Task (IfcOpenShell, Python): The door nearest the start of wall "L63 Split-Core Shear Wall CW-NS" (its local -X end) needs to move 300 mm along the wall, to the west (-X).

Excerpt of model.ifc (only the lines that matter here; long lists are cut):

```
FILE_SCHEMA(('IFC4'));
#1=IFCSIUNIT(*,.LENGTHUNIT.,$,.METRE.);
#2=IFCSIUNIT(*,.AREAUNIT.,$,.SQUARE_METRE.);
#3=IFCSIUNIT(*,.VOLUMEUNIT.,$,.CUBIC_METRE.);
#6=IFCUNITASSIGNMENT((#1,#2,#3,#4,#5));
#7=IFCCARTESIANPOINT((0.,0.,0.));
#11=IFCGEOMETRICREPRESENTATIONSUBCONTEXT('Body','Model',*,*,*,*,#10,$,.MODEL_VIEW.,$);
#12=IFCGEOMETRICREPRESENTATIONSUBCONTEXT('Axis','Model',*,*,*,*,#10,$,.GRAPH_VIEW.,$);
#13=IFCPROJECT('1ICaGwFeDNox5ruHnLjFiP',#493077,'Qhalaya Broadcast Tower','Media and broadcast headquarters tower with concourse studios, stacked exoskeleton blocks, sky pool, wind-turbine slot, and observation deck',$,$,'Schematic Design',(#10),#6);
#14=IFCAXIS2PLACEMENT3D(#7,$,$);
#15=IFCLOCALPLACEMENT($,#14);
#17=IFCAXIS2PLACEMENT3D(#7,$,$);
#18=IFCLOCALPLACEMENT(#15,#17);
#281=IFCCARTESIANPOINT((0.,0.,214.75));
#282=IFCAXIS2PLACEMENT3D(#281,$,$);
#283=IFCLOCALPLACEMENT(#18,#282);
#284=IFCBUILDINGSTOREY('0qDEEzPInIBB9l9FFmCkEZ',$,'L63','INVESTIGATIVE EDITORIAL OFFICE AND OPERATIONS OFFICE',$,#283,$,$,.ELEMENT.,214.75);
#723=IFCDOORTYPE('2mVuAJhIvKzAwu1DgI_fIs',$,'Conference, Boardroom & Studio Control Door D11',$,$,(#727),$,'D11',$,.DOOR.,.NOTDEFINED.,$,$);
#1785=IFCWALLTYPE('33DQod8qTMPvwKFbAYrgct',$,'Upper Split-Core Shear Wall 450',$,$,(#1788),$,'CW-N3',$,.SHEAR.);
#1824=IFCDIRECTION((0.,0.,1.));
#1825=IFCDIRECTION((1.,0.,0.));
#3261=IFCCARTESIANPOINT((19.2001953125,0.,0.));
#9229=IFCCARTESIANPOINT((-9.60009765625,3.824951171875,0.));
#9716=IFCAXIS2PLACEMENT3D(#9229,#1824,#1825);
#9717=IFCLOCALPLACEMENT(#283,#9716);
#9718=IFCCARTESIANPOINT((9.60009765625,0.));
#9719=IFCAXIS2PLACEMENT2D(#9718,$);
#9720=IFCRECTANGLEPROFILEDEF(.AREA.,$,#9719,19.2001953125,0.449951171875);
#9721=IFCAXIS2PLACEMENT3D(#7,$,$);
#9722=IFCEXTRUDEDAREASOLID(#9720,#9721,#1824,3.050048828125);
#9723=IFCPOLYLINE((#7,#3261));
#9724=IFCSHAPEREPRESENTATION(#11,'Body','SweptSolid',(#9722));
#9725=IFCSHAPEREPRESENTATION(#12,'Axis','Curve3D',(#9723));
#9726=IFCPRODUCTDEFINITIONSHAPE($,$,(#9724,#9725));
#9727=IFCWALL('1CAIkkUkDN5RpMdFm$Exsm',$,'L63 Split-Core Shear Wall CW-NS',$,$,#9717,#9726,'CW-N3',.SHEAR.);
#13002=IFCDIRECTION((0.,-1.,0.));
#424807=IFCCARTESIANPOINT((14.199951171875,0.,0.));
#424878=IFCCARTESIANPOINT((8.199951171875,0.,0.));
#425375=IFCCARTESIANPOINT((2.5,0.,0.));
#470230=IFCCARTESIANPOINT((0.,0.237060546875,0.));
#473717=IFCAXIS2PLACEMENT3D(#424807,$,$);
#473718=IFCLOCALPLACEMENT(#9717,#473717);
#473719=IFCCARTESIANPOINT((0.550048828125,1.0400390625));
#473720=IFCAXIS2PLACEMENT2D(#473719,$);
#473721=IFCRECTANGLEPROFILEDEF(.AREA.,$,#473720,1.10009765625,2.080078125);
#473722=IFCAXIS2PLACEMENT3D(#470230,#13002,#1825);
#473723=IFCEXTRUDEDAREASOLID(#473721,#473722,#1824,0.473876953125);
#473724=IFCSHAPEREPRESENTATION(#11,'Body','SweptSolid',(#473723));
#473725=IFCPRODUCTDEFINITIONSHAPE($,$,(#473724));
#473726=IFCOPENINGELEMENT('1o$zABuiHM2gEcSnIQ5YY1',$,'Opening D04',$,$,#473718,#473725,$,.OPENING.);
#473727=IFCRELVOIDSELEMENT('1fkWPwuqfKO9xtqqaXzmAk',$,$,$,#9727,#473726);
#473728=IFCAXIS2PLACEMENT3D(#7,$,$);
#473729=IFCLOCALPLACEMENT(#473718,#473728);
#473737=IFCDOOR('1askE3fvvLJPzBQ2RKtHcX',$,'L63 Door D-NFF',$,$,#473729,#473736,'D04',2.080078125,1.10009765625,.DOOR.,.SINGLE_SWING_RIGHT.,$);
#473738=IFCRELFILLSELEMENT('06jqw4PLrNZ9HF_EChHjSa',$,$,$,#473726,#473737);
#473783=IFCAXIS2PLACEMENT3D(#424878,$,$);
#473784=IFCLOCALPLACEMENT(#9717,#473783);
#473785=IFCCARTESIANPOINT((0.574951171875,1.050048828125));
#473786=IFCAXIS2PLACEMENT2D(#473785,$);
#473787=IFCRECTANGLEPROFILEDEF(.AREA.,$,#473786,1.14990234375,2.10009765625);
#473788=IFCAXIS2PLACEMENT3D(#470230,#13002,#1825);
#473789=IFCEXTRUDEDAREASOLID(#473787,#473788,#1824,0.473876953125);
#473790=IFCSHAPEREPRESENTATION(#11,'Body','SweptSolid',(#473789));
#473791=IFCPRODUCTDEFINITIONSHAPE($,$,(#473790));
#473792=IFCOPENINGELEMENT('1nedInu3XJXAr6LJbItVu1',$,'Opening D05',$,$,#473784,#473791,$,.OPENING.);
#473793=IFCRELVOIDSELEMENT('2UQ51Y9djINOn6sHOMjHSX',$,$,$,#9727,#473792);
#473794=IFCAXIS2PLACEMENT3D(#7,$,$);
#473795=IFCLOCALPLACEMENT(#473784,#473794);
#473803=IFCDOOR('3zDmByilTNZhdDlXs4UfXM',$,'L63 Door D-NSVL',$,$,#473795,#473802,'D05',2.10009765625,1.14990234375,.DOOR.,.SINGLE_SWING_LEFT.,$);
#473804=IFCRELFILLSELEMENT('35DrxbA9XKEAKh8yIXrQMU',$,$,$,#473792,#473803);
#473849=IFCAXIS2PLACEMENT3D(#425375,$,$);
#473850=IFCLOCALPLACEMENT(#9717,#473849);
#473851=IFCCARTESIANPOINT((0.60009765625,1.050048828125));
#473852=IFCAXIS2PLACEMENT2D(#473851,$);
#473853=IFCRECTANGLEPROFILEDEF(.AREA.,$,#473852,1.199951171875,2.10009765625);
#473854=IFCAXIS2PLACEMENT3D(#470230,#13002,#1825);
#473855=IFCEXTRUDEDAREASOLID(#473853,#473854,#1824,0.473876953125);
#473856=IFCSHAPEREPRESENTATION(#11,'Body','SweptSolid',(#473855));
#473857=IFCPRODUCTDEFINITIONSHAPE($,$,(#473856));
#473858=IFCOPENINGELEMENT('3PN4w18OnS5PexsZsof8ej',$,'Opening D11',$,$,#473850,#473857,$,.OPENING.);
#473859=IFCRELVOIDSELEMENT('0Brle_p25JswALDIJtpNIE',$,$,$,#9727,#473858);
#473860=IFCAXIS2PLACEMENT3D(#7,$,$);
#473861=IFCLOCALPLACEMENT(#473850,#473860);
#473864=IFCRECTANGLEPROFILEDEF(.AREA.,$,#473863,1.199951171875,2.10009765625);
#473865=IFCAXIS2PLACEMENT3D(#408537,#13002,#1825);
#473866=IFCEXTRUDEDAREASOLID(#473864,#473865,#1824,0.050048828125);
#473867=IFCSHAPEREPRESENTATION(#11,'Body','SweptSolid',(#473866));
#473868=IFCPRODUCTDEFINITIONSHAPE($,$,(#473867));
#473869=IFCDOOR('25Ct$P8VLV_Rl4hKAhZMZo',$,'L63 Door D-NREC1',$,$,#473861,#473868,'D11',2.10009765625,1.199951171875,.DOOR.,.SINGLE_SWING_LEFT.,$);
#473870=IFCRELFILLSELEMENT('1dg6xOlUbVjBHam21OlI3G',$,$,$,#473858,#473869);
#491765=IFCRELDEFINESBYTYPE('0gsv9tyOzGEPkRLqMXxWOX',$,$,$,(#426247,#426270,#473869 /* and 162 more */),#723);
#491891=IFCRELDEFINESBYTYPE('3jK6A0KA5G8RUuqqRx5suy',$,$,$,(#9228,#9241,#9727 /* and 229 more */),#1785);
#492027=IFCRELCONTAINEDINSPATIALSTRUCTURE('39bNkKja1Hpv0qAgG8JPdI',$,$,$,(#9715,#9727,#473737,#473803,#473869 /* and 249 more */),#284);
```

```python
import ifcopenshell
import ifcopenshell.api.geometry
import ifcopenshell.util.placement
import ifcopenshell.util.unit

model = ifcopenshell.open("model.ifc")
unit_scale = ifcopenshell.util.unit.calculate_unit_scale(model)

door = model.by_guid("25Ct$P8VLV_Rl4hKAhZMZo")
opening = door.FillsVoids[0].RelatingOpeningElement
wall = opening.VoidsElements[0].RelatingBuildingElement

wall_matrix = ifcopenshell.util.placement.get_local_placement(wall.ObjectPlacement)
shift = wall_matrix[:3, 0] * -0.3 / unit_scale
before = ifcopenshell.util.placement.get_local_placement(door.ObjectPlacement)[:3, 3].copy()

# The door is placed relative to its opening, so it follows when the opening moves.
matrix = ifcopenshell.util.placement.get_local_placement(opening.ObjectPlacement)
matrix[:3, 3] += shift
ifcopenshell.api.geometry.edit_object_placement(
    model, product=opening, matrix=matrix, is_si=False, should_transform_children=True
)

after = ifcopenshell.util.placement.get_local_placement(door.ObjectPlacement)[:3, 3]
print("door moved by", (after - before).round(3) + 0.0)

model.write("model_rev.ifc")
```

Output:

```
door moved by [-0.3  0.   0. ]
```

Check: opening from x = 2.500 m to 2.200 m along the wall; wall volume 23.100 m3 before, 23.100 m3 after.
